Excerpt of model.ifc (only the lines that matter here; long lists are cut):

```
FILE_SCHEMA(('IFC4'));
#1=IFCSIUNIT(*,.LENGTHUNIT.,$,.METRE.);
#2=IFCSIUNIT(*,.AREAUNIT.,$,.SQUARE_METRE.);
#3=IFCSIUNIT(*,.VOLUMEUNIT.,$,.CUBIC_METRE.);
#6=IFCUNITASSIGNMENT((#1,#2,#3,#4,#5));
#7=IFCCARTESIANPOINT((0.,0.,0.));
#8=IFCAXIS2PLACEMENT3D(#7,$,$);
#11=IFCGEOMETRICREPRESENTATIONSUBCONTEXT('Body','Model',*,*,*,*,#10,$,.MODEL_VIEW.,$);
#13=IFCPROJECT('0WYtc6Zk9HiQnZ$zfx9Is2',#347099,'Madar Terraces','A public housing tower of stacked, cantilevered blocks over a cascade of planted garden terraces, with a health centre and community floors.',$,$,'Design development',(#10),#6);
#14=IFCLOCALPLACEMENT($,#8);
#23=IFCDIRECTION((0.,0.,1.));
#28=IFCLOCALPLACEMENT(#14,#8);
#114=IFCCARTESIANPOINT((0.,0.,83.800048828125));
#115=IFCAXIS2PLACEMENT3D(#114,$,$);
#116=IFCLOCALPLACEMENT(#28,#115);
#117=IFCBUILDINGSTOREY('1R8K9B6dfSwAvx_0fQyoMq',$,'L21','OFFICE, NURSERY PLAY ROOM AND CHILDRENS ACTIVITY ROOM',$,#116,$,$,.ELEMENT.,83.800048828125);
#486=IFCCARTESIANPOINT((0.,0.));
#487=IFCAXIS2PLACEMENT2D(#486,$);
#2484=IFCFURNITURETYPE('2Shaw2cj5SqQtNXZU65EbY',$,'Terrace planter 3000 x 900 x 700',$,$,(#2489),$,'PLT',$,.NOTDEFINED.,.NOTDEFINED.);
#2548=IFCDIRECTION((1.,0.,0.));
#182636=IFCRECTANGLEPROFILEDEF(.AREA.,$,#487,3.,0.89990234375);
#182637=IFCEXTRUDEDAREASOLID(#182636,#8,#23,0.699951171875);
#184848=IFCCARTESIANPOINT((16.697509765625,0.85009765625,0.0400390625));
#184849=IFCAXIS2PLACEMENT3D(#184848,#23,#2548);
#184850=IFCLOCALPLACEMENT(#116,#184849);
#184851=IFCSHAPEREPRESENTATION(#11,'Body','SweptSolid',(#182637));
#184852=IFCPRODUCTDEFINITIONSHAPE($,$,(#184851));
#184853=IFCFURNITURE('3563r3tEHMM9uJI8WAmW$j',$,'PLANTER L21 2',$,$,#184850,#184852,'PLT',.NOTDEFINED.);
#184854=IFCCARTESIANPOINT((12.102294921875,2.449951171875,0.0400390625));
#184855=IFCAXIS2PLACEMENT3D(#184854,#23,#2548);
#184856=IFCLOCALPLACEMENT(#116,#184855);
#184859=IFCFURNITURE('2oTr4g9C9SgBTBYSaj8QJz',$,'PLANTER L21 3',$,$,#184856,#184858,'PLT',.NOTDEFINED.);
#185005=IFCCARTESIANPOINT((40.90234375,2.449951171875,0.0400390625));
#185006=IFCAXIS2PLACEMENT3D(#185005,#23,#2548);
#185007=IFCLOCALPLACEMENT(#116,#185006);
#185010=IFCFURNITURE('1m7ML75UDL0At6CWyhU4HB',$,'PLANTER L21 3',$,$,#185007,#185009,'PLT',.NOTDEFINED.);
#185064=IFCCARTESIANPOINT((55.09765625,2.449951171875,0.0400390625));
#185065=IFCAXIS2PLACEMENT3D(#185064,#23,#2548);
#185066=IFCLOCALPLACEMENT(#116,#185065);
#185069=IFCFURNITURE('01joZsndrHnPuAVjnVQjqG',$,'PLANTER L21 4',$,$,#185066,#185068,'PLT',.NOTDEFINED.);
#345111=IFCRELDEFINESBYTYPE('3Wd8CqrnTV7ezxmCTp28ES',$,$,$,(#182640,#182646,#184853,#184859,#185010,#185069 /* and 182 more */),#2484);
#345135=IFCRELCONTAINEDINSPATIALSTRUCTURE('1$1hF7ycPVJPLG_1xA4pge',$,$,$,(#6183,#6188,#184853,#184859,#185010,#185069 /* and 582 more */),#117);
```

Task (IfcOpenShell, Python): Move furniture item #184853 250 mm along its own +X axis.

```python
import ifcopenshell
import ifcopenshell.api.geometry
import ifcopenshell.util.placement
import ifcopenshell.util.unit

model = ifcopenshell.open("model.ifc")
unit_scale = ifcopenshell.util.unit.calculate_unit_scale(model)

item = model.by_guid("3563r3tEHMM9uJI8WAmW$j")
matrix = ifcopenshell.util.placement.get_local_placement(item.ObjectPlacement)
matrix[:3, 3] += matrix[:3, 0] * 0.25 / unit_scale
ifcopenshell.api.geometry.edit_object_placement(model, product=item, matrix=matrix, is_si=False)

print(ifcopenshell.util.placement.get_local_placement(item.ObjectPlacement).round(3) + 0.0)

model.write("model-out.ifc")
```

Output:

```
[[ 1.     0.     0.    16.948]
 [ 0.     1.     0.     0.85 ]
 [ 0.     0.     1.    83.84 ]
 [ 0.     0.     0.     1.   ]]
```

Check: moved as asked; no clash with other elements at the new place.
